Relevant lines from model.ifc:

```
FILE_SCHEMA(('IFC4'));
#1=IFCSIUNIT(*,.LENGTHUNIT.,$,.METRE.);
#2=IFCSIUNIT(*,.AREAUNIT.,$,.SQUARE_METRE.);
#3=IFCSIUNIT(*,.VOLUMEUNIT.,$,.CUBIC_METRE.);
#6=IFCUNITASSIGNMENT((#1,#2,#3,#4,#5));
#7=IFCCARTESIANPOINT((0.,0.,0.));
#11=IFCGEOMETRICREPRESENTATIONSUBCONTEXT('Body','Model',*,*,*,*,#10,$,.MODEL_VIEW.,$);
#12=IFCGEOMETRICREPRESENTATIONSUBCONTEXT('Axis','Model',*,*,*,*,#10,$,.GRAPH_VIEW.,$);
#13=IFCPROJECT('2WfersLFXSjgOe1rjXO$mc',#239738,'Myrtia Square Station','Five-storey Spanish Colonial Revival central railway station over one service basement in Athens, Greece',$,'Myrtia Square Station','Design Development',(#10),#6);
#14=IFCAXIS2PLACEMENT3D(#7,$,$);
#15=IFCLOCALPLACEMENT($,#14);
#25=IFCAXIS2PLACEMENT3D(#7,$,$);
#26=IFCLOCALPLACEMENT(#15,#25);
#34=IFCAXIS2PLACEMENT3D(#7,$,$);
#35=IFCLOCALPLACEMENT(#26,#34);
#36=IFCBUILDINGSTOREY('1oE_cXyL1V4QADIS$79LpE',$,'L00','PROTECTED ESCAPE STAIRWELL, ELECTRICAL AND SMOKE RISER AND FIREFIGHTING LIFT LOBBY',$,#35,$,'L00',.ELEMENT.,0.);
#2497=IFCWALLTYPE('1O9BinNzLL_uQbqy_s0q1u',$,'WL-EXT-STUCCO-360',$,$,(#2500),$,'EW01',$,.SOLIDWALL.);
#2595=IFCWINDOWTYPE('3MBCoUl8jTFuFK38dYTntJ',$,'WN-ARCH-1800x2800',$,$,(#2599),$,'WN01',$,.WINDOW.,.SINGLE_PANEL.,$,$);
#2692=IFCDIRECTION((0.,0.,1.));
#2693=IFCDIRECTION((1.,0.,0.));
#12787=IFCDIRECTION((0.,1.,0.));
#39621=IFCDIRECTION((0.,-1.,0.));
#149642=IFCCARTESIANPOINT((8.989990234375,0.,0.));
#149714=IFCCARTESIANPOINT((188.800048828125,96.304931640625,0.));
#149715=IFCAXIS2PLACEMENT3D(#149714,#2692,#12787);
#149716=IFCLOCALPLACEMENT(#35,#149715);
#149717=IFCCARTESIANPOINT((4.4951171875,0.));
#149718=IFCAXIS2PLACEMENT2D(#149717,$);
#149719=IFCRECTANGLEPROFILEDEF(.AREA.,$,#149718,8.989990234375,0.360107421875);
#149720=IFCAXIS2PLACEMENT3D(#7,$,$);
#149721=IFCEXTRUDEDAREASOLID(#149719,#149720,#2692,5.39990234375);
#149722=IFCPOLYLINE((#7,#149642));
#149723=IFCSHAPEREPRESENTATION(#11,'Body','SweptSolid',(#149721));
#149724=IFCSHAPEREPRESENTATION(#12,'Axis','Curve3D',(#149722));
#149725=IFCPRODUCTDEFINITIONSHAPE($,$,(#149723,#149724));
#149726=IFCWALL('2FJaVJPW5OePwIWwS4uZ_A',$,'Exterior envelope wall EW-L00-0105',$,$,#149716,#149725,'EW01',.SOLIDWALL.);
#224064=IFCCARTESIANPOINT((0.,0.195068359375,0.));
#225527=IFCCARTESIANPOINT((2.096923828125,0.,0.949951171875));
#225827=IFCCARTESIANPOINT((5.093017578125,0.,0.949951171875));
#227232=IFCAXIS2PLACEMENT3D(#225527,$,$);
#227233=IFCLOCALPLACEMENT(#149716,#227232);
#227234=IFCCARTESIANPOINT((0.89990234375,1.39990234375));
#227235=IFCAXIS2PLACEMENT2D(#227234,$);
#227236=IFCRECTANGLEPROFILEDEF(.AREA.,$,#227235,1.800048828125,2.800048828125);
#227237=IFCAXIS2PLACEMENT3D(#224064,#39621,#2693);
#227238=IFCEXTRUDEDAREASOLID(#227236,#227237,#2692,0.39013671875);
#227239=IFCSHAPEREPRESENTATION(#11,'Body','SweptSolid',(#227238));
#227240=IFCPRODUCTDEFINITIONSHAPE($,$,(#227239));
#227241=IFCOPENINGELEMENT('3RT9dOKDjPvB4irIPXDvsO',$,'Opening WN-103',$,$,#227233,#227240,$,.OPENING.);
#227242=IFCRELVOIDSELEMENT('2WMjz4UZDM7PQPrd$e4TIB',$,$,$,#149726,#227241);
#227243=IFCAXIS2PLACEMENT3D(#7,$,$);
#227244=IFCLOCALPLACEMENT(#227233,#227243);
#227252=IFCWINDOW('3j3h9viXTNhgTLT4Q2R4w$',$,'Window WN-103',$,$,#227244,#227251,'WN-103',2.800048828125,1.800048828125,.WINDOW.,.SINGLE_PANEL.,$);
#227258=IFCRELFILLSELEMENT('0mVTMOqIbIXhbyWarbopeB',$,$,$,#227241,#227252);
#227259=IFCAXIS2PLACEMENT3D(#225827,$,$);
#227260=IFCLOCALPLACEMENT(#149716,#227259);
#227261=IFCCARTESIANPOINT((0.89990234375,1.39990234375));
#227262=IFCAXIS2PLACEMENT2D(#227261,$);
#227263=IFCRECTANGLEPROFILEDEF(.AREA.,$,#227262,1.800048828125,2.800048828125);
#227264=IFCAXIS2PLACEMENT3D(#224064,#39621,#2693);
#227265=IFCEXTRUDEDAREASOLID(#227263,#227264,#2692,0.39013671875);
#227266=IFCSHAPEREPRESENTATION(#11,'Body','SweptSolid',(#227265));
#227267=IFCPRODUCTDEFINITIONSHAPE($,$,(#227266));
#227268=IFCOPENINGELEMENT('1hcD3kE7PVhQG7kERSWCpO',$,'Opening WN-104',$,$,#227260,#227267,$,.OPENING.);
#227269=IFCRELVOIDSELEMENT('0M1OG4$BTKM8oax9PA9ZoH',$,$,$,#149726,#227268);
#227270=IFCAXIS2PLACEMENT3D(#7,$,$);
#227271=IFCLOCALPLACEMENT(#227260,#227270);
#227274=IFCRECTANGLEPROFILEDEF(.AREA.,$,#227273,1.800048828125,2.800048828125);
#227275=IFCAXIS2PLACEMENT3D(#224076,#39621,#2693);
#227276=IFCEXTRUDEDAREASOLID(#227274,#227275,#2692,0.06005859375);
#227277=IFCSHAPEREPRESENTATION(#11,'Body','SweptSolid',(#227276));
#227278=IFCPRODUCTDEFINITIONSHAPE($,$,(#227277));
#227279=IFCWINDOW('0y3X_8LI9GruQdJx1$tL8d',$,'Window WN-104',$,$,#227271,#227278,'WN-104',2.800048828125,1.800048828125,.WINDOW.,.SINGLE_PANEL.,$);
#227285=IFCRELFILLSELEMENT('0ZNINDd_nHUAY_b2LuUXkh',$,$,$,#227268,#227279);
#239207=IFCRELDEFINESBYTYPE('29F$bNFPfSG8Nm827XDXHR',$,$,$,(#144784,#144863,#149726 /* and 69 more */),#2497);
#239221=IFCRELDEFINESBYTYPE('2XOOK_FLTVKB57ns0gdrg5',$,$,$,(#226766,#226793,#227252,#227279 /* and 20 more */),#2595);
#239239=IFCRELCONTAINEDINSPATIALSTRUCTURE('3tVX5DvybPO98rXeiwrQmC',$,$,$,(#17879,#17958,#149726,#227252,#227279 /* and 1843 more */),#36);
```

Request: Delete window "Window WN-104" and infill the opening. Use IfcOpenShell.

```python
import ifcopenshell
import ifcopenshell.api.feature
import ifcopenshell.api.root
import ifcopenshell.geom
import ifcopenshell.util.shape

model = ifcopenshell.open("model.ifc")
settings = ifcopenshell.geom.settings()


def volume(element):
    """Net volume in cubic metres, openings subtracted."""
    shape = ifcopenshell.geom.create_shape(settings, element)
    return ifcopenshell.util.shape.get_volume(shape.geometry)


window = model.by_id(227279)
opening = window.FillsVoids[0].RelatingOpeningElement
wall = opening.VoidsElements[0].RelatingBuildingElement
before = volume(wall)

ifcopenshell.api.root.remove_product(model, product=window)
ifcopenshell.api.feature.remove_feature(model, feature=opening)

after = volume(wall)

print(f"wall volume {before:.3f} -> {after:.3f} m3")

model.write("model-out.ifc")
```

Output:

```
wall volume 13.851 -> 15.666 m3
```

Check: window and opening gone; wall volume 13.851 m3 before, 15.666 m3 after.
